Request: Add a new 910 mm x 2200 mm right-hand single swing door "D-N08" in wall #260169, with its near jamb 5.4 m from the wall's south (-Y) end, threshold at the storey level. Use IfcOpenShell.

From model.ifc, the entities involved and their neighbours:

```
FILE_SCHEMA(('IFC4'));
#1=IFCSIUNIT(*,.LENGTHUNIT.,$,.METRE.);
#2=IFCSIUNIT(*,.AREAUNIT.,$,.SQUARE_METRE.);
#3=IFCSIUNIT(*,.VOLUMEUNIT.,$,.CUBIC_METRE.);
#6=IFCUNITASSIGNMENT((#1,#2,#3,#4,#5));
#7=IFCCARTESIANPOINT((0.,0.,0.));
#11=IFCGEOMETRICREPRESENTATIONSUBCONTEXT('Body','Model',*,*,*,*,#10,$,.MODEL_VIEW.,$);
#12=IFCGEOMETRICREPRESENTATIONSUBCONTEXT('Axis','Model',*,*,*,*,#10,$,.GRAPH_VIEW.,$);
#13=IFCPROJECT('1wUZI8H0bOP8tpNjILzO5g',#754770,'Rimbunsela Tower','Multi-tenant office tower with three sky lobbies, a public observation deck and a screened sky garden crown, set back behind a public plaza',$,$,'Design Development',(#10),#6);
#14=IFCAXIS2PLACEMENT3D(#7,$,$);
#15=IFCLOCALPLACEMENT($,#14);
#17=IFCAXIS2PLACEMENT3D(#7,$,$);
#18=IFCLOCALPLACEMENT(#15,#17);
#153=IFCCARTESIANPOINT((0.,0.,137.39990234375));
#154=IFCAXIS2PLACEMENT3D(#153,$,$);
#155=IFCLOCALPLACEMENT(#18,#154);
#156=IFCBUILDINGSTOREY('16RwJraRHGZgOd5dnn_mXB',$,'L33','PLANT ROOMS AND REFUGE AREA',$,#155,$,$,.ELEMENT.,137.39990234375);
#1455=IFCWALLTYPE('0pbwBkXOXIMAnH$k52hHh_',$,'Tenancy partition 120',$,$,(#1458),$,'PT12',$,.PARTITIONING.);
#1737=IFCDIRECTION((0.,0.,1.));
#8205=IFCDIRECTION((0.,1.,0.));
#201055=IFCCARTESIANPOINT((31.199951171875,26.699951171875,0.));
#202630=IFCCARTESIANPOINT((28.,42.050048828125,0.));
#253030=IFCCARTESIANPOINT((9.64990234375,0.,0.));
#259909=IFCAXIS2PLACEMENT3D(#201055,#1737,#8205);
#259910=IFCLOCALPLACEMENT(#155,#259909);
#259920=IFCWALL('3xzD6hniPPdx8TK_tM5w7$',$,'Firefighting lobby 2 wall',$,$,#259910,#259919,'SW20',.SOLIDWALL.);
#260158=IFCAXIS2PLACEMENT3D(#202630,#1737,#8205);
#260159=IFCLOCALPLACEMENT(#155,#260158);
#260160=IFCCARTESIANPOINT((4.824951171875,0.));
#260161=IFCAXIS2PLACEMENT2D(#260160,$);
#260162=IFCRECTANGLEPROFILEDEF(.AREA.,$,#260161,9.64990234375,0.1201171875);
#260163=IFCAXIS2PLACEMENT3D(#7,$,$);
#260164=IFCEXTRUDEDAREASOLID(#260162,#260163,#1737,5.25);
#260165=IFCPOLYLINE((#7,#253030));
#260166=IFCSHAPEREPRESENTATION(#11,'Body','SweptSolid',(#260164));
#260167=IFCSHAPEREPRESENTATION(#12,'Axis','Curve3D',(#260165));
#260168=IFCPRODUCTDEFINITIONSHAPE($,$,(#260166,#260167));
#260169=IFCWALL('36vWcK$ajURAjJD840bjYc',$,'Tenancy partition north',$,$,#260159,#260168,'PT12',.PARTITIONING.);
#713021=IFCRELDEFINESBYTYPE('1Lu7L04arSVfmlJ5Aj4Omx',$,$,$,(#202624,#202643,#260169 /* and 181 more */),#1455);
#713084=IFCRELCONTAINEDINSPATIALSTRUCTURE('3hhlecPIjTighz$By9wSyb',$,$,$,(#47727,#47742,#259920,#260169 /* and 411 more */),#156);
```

```python
import numpy as np
import ifcopenshell
import ifcopenshell.api.feature
import ifcopenshell.api.geometry
import ifcopenshell.api.root
import ifcopenshell.api.spatial
import ifcopenshell.geom
import ifcopenshell.util.element
import ifcopenshell.util.placement
import ifcopenshell.util.representation
import ifcopenshell.util.shape
import ifcopenshell.util.unit

model = ifcopenshell.open("model.ifc")
unit_scale = ifcopenshell.util.unit.calculate_unit_scale(model)
settings = ifcopenshell.geom.settings()


def volume(element):
    """Net volume in cubic metres, openings subtracted."""
    shape = ifcopenshell.geom.create_shape(settings, element)
    return ifcopenshell.util.shape.get_volume(shape.geometry)


wall = model.by_id(260169)
storey = ifcopenshell.util.element.get_container(wall, ifc_class="IfcBuildingStorey")
context = ifcopenshell.util.representation.get_context(model, "Model", "Body", "MODEL_VIEW")
before = volume(wall)

width, height, from_end, sill = 0.91, 2.2, 5.4, 0.0  # metres

# The wall runs along its own X axis, and the end named is its -X end.
wall_shape = ifcopenshell.geom.create_shape(settings, wall)
x, y, z = ifcopenshell.util.shape.get_vertices(wall_shape.geometry).T
start = x.min() + from_end
face, thickness = float(y.min()), float(y.max() - y.min())
wall_matrix = ifcopenshell.util.placement.get_local_placement(wall.ObjectPlacement)
level = ifcopenshell.util.placement.get_local_placement(storey.ObjectPlacement)[2, 3]


def in_wall(x, y):
    """Placement at x, y metres in the wall's axes, at sill height."""
    matrix = wall_matrix.copy()
    matrix[:, 3] = wall_matrix @ np.array([x / unit_scale, y / unit_scale, 0.0, 1.0])
    matrix[2, 3] = level + sill / unit_scale
    return matrix


# Opening: a box that overshoots both wall faces by 50 mm.
opening = ifcopenshell.api.root.create_entity(model, ifc_class="IfcOpeningElement", predefined_type="OPENING")
box = ifcopenshell.api.geometry.add_wall_representation(
    model, context=context, length=width, height=height, thickness=thickness + 0.1
)
ifcopenshell.api.geometry.assign_representation(model, product=opening, representation=box)
ifcopenshell.api.geometry.edit_object_placement(model, product=opening, matrix=in_wall(start, face - 0.05), is_si=False)
ifcopenshell.api.feature.add_feature(model, feature=opening, element=wall)

door = ifcopenshell.api.root.create_entity(model, ifc_class="IfcDoor", name="D-N08", predefined_type="DOOR")
door.OverallWidth, door.OverallHeight = width / unit_scale, height / unit_scale
door.OperationType = "SINGLE_SWING_RIGHT"
body = ifcopenshell.api.geometry.add_door_representation(
    model,
    context=context,
    overall_width=door.OverallWidth,
    overall_height=door.OverallHeight,
    operation_type="SINGLE_SWING_RIGHT",
    lining_properties={"LiningDepth": thickness / unit_scale, "ThresholdDepth": thickness / unit_scale},
)
ifcopenshell.api.geometry.assign_representation(model, product=door, representation=body)
ifcopenshell.api.spatial.assign_container(model, products=[door], relating_structure=storey)
ifcopenshell.api.feature.add_filling(model, opening=opening, element=door)

# The lining spans the wall, so the door starts at the wall face.
ifcopenshell.api.geometry.edit_object_placement(model, product=door, matrix=in_wall(start, face), is_si=False)

after = volume(wall)

print(f"wall volume {before:.3f} -> {after:.3f} m3")

model.write("model_v2.ifc")
```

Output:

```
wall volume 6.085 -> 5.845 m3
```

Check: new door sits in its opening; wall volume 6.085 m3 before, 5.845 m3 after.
